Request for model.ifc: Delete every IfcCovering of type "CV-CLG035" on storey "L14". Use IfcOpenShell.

First a look at what the model holds.

```python
import ifcopenshell
import ifcopenshell.util.element

model = ifcopenshell.open("model.ifc")
print(model.schema)
storey = next(s for s in model.by_type("IfcBuildingStorey") if s.Name == "L14")
coverings = [e for e in ifcopenshell.util.element.get_decomposition(storey) if e.is_a("IfcCovering")]
seen = {}
for e in coverings:
    element_type = ifcopenshell.util.element.get_type(e)
    name = element_type.Name if element_type not in (None, e) else None
    seen[name] = seen.get(name, 0) + 1
for name, count in sorted(seen.items(), key=str):
    print(count, "x", name)
```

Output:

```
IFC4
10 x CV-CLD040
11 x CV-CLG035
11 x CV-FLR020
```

```python
import ifcopenshell
import ifcopenshell.api.root
import ifcopenshell.util.element

model = ifcopenshell.open("model.ifc")

storey = next(s for s in model.by_type("IfcBuildingStorey") if s.Name == "L14")
coverings = [e for e in ifcopenshell.util.element.get_decomposition(storey) if e.is_a("IfcCovering")]
targets = [e for e in coverings if (t := ifcopenshell.util.element.get_type(e)) not in (None, e) and t.Name == "CV-CLG035"]

for e in targets:
    ifcopenshell.api.root.remove_product(model, product=e)
print(len(targets), "removed")

model.write("model_updated.ifc")
```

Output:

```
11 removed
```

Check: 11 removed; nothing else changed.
